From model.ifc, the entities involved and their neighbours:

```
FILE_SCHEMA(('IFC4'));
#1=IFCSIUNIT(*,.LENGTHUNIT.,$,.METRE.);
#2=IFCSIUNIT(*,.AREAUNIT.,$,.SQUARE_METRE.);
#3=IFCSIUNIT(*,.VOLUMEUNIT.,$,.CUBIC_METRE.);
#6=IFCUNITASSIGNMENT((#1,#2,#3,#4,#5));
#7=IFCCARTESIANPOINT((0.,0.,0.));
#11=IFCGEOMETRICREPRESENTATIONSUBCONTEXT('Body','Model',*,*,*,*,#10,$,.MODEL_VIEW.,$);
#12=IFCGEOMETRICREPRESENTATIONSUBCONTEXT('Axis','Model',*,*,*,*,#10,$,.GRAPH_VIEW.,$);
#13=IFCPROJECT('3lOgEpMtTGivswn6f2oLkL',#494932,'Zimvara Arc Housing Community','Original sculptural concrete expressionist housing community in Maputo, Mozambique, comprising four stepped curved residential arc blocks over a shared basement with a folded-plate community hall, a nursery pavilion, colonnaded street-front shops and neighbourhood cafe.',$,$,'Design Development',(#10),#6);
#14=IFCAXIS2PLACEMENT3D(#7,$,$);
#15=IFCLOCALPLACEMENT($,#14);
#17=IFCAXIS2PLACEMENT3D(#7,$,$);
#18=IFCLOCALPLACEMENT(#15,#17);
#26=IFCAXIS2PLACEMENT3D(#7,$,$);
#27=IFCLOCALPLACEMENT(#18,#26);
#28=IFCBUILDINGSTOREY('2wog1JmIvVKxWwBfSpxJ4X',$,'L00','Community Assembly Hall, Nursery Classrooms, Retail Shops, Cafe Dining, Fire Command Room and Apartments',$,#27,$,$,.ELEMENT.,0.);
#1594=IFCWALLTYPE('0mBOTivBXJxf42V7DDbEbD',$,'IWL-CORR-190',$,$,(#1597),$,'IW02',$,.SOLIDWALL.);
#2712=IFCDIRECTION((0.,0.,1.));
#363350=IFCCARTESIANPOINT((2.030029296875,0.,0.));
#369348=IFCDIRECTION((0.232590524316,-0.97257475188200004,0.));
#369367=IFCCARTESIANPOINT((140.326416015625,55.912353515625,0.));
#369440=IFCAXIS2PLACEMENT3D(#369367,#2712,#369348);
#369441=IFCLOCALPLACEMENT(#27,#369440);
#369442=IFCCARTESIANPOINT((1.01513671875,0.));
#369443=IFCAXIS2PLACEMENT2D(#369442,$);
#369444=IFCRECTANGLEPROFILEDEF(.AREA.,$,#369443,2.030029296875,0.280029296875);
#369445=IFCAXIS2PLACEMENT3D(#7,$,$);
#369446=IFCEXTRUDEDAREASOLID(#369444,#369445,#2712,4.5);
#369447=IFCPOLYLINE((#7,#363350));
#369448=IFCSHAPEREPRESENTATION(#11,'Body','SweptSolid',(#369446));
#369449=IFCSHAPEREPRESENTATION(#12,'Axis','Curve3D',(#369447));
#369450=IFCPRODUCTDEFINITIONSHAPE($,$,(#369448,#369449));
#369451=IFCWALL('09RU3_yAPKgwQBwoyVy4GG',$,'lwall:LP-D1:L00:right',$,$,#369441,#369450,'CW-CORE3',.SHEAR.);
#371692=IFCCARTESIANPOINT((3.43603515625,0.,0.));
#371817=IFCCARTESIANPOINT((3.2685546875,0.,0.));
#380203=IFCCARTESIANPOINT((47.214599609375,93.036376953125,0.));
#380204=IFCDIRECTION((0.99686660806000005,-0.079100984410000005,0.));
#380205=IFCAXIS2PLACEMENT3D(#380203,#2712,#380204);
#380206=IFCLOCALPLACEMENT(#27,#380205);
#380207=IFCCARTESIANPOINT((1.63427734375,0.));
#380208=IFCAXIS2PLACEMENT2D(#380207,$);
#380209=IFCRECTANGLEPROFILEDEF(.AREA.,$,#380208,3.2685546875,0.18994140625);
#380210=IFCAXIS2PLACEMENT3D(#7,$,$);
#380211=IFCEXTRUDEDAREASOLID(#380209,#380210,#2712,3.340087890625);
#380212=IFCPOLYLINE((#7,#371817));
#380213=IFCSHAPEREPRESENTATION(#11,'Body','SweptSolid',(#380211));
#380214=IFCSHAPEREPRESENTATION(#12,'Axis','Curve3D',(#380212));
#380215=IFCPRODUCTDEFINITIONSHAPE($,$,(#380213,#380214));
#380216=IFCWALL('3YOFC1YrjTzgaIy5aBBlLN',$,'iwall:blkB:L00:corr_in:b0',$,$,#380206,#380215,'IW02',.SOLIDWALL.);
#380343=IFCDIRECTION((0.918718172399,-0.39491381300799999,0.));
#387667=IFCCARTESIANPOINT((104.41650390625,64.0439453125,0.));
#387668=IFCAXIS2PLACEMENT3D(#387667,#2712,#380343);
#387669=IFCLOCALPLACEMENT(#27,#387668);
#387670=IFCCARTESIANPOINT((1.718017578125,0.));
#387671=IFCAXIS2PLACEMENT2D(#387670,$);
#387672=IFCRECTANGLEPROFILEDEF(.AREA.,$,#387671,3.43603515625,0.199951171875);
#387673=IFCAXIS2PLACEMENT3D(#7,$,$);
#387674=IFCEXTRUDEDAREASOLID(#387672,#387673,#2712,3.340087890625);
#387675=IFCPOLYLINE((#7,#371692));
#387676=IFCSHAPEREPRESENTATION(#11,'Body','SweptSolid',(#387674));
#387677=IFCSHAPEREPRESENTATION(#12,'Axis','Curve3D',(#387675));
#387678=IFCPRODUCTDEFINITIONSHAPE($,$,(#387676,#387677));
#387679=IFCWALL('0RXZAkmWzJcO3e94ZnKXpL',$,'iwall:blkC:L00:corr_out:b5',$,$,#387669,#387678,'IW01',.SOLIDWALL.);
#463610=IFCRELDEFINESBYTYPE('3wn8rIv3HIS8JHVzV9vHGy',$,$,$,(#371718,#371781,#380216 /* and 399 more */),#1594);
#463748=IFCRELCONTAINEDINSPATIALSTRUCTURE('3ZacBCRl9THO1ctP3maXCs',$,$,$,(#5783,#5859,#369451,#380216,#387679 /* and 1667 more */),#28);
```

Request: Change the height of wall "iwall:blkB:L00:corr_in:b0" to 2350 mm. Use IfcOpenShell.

```python
import ifcopenshell
import ifcopenshell.geom
import ifcopenshell.util.representation
import ifcopenshell.util.shape
import ifcopenshell.util.unit

model = ifcopenshell.open("model.ifc")
unit_scale = ifcopenshell.util.unit.calculate_unit_scale(model)
settings = ifcopenshell.geom.settings()


def volume(element):
    """Net volume in cubic metres, openings subtracted."""
    shape = ifcopenshell.geom.create_shape(settings, element)
    return ifcopenshell.util.shape.get_volume(shape.geometry)


wall = model.by_guid("3YOFC1YrjTzgaIy5aBBlLN")
before = volume(wall)

body = ifcopenshell.util.representation.get_representation(wall, "Model", "Body")
solid = body.Items[0]
old_height = solid.Depth
solid.Depth = 2.35 / unit_scale
after = volume(wall)

print(f"height {old_height:g} -> {solid.Depth:g}, volume {before:.3f} -> {after:.3f} m3")

model.write("model_v2.ifc")
```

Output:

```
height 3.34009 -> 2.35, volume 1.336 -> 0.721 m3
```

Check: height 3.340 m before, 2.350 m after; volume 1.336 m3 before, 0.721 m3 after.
